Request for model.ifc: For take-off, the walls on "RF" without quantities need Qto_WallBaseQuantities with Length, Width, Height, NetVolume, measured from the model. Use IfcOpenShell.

First a look at what the model holds.

```python
import ifcopenshell
import ifcopenshell.util.element
import ifcopenshell.util.unit

model = ifcopenshell.open("model.ifc")
print(model.schema)
for unit_type in ("LENGTHUNIT", "AREAUNIT", "VOLUMEUNIT"):
    print(unit_type, ifcopenshell.util.unit.calculate_unit_scale(model, unit_type))
storey = next(s for s in model.by_type("IfcBuildingStorey") if s.Name == "RF")
walls = [e for e in ifcopenshell.util.element.get_decomposition(storey) if e.is_a("IfcWall")]
for e in sorted(walls, key=lambda e: e.id()):
    print(e.id(), e.is_a(), e.Name, list(ifcopenshell.util.element.get_psets(e, qtos_only=True)), sep=" | ")
```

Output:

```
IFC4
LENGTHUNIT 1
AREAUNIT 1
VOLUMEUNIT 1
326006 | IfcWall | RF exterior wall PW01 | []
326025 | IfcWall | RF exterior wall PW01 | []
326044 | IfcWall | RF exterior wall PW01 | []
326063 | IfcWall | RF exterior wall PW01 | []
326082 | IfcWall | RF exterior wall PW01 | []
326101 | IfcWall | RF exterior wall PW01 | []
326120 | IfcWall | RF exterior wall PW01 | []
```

```python
import ifcopenshell
import ifcopenshell.api.pset
import ifcopenshell.geom
import ifcopenshell.util.element
import ifcopenshell.util.shape
import ifcopenshell.util.unit

model = ifcopenshell.open("model.ifc")
unit_scale = ifcopenshell.util.unit.calculate_unit_scale(model)
volume_scale = ifcopenshell.util.unit.calculate_unit_scale(model, "VOLUMEUNIT")
settings = ifcopenshell.geom.settings()

storey = next(s for s in model.by_type("IfcBuildingStorey") if s.Name == "RF")
walls = [e for e in ifcopenshell.util.element.get_decomposition(storey) if e.is_a("IfcWall")]

for e in sorted(walls, key=lambda e: e.id()):
    if ifcopenshell.util.element.get_psets(e, qtos_only=True, should_inherit=False):
        continue
    # Geometry comes back in metres, in the element's own axes.
    shape = ifcopenshell.geom.create_shape(settings, e)
    values = {
        "Length": ifcopenshell.util.shape.get_x(shape.geometry) / unit_scale,
        "Width": ifcopenshell.util.shape.get_y(shape.geometry) / unit_scale,
        "Height": ifcopenshell.util.shape.get_z(shape.geometry) / unit_scale,
        "NetVolume": ifcopenshell.util.shape.get_volume(shape.geometry) / volume_scale,
    }
    qto = ifcopenshell.api.pset.add_qto(model, product=e, name="Qto_WallBaseQuantities")
    ifcopenshell.api.pset.edit_qto(model, qto=qto, properties=values)
    print(e.id(), {k: round(v, 3) for k, v in values.items()})

model.write("model_v2.ifc")
```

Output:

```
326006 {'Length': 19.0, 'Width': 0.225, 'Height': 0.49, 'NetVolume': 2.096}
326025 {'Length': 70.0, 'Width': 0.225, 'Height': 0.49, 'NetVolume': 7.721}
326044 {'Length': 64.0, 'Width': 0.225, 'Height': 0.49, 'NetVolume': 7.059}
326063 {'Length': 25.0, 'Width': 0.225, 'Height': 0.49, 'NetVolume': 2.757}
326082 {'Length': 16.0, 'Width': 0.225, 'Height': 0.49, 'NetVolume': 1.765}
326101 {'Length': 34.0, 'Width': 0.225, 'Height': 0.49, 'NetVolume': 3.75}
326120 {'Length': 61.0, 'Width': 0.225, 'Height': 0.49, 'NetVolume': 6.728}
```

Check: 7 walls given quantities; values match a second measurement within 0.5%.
